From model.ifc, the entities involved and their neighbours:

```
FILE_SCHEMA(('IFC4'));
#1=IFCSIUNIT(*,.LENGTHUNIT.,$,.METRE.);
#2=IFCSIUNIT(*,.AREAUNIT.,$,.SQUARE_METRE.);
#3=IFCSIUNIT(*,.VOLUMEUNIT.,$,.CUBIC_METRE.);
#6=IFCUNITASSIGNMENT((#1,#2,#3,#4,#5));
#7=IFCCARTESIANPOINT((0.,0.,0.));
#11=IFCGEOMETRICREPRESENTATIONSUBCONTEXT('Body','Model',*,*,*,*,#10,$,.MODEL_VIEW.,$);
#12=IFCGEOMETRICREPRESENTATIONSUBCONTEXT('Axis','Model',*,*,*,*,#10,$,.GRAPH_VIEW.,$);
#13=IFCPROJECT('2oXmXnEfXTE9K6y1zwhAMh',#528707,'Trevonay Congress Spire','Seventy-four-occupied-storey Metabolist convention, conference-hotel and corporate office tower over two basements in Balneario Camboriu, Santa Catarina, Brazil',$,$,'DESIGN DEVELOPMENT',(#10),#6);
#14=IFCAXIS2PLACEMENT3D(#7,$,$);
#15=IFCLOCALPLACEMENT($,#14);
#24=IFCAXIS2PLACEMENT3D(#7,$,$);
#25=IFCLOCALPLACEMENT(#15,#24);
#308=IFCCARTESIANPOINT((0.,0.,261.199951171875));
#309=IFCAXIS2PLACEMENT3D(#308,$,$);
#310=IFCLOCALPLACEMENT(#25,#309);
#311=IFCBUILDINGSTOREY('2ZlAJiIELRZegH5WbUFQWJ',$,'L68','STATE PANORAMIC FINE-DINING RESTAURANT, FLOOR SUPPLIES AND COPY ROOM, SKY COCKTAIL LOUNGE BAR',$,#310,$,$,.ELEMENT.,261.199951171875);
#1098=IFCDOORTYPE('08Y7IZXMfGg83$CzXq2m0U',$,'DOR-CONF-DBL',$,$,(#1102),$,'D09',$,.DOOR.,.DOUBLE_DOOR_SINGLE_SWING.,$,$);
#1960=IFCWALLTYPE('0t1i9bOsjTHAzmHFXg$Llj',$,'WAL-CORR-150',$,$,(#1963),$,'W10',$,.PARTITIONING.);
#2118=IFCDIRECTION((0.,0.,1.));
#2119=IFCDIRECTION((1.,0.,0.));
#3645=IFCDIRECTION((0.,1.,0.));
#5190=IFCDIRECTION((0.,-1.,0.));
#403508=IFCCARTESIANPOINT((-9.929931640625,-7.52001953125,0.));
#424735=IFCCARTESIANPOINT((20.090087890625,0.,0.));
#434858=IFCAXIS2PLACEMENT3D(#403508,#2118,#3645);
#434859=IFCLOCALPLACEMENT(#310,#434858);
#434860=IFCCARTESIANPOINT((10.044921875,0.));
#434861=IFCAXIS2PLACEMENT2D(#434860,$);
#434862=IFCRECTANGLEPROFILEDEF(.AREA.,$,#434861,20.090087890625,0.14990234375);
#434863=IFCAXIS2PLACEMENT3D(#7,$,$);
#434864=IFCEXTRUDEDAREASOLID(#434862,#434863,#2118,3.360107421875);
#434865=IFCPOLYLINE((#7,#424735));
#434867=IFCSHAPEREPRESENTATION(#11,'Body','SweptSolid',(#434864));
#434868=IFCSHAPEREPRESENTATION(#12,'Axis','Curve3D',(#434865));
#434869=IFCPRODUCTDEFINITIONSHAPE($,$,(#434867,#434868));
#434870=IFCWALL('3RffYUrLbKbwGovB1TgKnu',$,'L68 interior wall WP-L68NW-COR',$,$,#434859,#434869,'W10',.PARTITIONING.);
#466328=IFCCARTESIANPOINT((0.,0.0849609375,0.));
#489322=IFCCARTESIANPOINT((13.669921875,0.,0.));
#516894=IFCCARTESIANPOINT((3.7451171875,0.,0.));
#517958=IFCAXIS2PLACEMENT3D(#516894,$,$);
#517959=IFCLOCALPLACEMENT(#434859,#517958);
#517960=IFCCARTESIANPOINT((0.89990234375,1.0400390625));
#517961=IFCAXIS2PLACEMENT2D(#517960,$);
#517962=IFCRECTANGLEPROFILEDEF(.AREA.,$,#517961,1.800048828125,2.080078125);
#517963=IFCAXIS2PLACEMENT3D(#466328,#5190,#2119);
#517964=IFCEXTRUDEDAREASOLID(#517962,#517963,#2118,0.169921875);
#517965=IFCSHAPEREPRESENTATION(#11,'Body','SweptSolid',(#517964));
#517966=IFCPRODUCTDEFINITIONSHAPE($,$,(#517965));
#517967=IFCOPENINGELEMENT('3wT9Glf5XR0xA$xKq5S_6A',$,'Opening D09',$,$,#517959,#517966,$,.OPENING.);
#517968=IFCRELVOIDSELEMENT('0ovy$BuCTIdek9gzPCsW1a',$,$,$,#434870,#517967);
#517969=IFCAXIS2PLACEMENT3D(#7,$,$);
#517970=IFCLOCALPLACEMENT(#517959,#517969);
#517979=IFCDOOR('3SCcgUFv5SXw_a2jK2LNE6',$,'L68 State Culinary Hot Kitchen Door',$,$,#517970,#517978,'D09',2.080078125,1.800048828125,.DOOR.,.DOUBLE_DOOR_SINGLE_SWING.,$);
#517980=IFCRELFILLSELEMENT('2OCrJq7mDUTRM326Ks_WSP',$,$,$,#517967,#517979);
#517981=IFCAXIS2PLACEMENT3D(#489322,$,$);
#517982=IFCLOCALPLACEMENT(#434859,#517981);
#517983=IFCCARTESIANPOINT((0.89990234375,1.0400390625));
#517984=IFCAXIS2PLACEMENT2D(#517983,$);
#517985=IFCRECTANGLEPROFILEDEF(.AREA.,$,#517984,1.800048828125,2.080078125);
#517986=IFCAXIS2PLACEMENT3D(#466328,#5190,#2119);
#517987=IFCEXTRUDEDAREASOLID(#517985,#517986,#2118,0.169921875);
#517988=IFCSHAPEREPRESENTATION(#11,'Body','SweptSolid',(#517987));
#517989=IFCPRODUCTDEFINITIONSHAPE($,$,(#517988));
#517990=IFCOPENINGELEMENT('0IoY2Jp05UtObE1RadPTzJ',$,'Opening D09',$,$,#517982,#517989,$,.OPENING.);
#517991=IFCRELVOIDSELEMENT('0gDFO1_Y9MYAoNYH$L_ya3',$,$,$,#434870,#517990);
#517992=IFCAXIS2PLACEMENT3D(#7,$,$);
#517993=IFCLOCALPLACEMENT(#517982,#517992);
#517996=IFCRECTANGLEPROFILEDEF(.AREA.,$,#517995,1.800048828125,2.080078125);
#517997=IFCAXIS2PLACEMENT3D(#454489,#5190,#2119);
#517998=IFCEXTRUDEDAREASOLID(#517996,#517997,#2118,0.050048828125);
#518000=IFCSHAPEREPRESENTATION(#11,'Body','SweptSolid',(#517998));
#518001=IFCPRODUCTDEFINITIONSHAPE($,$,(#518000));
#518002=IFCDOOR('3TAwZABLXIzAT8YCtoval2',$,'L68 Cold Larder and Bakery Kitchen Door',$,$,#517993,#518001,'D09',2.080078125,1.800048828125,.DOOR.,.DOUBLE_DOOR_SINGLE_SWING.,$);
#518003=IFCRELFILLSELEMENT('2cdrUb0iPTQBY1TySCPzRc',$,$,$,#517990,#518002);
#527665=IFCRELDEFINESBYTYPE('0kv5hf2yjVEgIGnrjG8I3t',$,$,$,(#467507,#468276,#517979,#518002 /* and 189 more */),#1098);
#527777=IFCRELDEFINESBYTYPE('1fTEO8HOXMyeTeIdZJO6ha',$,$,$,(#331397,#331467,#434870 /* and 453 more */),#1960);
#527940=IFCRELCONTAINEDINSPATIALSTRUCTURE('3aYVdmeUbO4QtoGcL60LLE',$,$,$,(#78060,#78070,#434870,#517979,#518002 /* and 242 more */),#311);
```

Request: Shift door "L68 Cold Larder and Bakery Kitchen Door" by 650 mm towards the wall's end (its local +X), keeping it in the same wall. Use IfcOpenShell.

```python
import ifcopenshell
import ifcopenshell.api.geometry
import ifcopenshell.util.placement
import ifcopenshell.util.unit

model = ifcopenshell.open("model.ifc")
unit_scale = ifcopenshell.util.unit.calculate_unit_scale(model)

door = model.by_guid("3TAwZABLXIzAT8YCtoval2")
opening = door.FillsVoids[0].RelatingOpeningElement
wall = opening.VoidsElements[0].RelatingBuildingElement

wall_matrix = ifcopenshell.util.placement.get_local_placement(wall.ObjectPlacement)
shift = wall_matrix[:3, 0] * 0.65 / unit_scale
before = ifcopenshell.util.placement.get_local_placement(door.ObjectPlacement)[:3, 3].copy()

# The door is placed relative to its opening, so it follows when the opening moves.
matrix = ifcopenshell.util.placement.get_local_placement(opening.ObjectPlacement)
matrix[:3, 3] += shift
ifcopenshell.api.geometry.edit_object_placement(
    model, product=opening, matrix=matrix, is_si=False, should_transform_children=True
)

after = ifcopenshell.util.placement.get_local_placement(door.ObjectPlacement)[:3, 3]
print("door moved by", (after - before).round(3) + 0.0)

model.write("model_updated.ifc")
```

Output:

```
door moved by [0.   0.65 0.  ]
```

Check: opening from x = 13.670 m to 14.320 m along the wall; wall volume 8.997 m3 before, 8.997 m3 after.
